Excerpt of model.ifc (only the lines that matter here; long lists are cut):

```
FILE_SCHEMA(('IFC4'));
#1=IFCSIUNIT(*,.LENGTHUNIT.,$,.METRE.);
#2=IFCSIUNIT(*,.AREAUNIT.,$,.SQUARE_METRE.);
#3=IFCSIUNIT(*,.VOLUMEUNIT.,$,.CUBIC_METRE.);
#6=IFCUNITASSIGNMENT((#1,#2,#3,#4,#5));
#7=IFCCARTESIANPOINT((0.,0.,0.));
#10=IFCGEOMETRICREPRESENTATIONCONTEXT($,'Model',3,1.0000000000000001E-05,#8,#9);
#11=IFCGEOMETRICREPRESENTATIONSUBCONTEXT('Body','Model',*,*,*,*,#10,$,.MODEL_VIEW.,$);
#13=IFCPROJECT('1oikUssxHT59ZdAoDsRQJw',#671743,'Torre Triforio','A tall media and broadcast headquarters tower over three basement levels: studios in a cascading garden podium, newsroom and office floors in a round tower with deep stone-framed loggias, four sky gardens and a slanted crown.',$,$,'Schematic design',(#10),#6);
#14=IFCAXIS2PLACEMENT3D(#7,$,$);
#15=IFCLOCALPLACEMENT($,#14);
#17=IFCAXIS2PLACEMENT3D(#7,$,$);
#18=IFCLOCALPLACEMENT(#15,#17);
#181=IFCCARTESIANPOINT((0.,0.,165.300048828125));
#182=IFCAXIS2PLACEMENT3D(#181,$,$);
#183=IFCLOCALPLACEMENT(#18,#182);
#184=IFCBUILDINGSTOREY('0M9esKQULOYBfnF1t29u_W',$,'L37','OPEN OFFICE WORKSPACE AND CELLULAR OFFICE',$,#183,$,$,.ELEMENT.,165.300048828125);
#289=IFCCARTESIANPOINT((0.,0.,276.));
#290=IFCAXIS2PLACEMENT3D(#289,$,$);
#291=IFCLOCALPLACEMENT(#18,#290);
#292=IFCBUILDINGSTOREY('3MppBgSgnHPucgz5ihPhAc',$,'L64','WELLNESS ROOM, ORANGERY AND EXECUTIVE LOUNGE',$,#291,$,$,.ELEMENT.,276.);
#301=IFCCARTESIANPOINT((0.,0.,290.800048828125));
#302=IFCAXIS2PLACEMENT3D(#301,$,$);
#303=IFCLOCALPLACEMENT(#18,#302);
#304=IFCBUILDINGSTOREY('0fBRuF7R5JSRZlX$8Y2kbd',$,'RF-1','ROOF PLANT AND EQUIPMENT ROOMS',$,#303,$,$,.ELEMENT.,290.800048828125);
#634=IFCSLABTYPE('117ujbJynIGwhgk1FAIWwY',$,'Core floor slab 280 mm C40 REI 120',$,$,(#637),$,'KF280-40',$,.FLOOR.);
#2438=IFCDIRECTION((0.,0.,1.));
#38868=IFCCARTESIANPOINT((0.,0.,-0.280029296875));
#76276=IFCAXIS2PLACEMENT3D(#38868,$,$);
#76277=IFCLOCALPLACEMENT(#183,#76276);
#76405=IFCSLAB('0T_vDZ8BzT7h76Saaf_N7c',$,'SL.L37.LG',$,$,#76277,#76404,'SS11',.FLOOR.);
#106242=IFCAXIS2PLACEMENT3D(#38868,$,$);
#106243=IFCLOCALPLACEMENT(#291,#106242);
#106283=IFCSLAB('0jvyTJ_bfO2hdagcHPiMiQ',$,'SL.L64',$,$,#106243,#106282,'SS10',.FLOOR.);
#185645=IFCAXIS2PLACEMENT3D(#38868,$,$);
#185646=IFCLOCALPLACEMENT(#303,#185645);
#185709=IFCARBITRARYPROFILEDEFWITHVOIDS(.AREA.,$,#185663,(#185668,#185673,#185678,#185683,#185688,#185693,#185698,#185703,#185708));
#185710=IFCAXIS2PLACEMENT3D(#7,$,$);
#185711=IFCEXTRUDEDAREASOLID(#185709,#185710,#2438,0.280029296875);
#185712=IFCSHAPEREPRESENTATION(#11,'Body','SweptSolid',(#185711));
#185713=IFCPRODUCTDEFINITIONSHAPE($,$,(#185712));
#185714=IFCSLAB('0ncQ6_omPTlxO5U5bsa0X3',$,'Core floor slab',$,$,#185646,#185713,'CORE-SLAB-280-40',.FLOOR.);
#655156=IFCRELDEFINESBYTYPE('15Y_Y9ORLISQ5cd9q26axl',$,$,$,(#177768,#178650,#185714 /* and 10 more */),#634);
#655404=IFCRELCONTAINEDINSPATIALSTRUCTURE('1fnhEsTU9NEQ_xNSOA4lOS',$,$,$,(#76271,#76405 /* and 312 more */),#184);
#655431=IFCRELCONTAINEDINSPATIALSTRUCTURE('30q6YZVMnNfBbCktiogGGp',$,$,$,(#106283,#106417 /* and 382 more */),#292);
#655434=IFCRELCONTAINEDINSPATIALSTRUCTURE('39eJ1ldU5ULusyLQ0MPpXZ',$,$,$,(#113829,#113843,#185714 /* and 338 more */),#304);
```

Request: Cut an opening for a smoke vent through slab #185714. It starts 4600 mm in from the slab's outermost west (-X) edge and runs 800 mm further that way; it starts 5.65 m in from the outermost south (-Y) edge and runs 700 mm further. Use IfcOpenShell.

```python
import numpy as np
import ifcopenshell
import ifcopenshell.api.feature
import ifcopenshell.api.geometry
import ifcopenshell.api.root
import ifcopenshell.geom
import ifcopenshell.util.placement
import ifcopenshell.util.representation
import ifcopenshell.util.shape
import ifcopenshell.util.unit

model = ifcopenshell.open("model.ifc")
unit_scale = ifcopenshell.util.unit.calculate_unit_scale(model)
settings = ifcopenshell.geom.settings()


def volume(element):
    """Net volume in cubic metres, openings subtracted."""
    shape = ifcopenshell.geom.create_shape(settings, element)
    return ifcopenshell.util.shape.get_volume(shape.geometry)


slab = model.by_guid("0ncQ6_omPTlxO5U5bsa0X3")
before = volume(slab)

# Extent in the slab's own axes, in metres. The edges named are its -X and -Y sides.
slab_shape = ifcopenshell.geom.create_shape(settings, slab)
vertices = ifcopenshell.util.shape.get_vertices(slab_shape.geometry)
x_min, y_min, bottom = vertices.min(axis=0)
top = vertices[:, 2].max()

opening = ifcopenshell.api.root.create_entity(model, ifc_class="IfcOpeningElement", name="Smoke vent opening", predefined_type="OPENING")
context = ifcopenshell.util.representation.get_context(model, "Model", "Body", "MODEL_VIEW")
width, depth = 0.8, 0.7
outline = [(0.0, 0.0), (width, 0.0), (width, depth), (0.0, depth), (0.0, 0.0)]
# Overshoot both faces by 50 mm so the cut is clean.
shape = ifcopenshell.api.geometry.add_slab_representation(
    model, context=context, depth=top - bottom + 0.1, polyline=outline
)
ifcopenshell.api.geometry.assign_representation(model, product=opening, representation=shape)

matrix = ifcopenshell.util.placement.get_local_placement(slab.ObjectPlacement)
matrix[:, 3] = matrix @ np.append(np.array([x_min + 4.6, y_min + 5.65, bottom - 0.05]) / unit_scale, 1.0)
ifcopenshell.api.geometry.edit_object_placement(model, product=opening, matrix=matrix, is_si=False)
ifcopenshell.api.feature.add_feature(model, feature=opening, element=slab)

after = volume(slab)

print(f"slab volume {before:.3f} -> {after:.3f} m3")

model.write("model_updated.ifc")
```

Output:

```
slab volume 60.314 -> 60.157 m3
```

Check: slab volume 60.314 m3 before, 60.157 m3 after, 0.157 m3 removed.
